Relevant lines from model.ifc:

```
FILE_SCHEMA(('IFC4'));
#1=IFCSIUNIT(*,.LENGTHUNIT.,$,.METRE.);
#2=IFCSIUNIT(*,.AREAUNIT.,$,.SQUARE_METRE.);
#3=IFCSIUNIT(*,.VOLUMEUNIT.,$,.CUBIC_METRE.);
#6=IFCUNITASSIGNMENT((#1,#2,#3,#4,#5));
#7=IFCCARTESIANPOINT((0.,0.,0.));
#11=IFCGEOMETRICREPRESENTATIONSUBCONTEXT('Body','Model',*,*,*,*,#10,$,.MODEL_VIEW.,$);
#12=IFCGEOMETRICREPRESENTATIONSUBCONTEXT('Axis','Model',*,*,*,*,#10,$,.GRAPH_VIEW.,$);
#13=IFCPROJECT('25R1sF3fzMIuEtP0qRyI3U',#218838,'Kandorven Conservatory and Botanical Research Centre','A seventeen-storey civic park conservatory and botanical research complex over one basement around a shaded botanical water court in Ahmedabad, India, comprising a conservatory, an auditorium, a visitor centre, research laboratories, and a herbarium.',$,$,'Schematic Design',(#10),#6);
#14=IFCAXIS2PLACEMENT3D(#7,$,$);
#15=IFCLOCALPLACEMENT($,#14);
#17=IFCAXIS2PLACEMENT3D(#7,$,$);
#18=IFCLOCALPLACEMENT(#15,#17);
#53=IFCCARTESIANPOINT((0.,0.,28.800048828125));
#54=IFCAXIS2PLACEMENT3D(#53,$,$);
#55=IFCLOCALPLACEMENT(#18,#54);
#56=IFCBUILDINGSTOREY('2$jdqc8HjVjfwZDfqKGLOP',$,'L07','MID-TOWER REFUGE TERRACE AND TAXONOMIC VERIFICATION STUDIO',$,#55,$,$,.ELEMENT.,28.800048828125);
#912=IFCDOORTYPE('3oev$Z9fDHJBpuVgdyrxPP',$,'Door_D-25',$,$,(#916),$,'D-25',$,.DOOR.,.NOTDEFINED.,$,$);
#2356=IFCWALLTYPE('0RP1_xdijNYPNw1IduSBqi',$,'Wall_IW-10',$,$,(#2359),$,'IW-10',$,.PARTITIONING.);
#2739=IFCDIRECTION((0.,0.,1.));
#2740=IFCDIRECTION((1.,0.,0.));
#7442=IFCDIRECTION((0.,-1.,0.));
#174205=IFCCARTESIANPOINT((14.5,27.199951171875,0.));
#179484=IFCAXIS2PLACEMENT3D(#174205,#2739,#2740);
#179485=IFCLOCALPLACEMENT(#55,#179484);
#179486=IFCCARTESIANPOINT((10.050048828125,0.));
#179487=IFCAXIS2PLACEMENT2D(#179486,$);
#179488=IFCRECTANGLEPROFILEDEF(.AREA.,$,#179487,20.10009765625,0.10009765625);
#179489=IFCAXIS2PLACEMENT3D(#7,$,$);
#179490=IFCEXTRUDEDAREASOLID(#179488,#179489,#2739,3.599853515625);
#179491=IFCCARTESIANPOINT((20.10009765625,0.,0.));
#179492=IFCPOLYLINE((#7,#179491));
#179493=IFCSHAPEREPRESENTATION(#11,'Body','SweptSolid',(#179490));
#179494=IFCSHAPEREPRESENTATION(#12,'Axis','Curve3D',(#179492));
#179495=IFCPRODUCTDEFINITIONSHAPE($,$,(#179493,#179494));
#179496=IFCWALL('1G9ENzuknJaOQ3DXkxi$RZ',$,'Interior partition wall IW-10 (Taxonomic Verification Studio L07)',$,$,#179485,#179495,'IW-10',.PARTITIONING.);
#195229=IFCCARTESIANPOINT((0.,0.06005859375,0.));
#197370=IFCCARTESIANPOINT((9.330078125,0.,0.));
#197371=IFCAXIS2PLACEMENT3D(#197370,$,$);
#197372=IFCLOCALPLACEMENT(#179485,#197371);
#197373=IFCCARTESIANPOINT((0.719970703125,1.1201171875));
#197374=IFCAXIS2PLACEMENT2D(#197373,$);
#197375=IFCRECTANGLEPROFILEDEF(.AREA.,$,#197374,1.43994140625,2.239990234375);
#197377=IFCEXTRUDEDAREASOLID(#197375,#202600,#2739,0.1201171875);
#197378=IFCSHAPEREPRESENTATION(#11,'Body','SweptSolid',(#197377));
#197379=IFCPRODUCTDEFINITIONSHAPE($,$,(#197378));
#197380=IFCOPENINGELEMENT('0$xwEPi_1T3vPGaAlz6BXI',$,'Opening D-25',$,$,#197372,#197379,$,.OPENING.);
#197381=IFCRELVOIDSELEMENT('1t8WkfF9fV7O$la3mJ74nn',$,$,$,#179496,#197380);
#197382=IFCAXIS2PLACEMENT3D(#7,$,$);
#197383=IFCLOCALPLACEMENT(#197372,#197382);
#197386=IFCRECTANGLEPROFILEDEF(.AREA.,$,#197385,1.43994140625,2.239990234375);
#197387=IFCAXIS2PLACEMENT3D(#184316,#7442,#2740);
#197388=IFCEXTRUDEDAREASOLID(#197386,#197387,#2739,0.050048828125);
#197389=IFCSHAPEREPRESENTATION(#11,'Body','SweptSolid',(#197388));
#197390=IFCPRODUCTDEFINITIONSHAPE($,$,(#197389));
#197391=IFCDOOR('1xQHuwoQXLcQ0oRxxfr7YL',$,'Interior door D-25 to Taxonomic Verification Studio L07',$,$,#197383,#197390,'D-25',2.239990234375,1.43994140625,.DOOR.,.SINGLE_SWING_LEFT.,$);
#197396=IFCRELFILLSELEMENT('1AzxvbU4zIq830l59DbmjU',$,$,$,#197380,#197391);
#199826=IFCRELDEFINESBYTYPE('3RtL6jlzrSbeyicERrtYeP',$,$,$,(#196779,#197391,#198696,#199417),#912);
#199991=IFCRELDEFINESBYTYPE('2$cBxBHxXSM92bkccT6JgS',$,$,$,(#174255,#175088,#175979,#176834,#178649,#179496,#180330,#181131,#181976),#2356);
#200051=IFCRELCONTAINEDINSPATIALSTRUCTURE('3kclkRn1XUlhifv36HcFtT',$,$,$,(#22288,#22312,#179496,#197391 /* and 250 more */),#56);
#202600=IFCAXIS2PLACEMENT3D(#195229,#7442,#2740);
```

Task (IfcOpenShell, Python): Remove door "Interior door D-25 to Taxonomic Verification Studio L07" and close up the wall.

```python
import ifcopenshell
import ifcopenshell.api.feature
import ifcopenshell.api.root
import ifcopenshell.geom
import ifcopenshell.util.shape

model = ifcopenshell.open("model.ifc")
settings = ifcopenshell.geom.settings()


def volume(element):
    """Net volume in cubic metres, openings subtracted."""
    shape = ifcopenshell.geom.create_shape(settings, element)
    return ifcopenshell.util.shape.get_volume(shape.geometry)


door = model.by_guid("1xQHuwoQXLcQ0oRxxfr7YL")
opening = door.FillsVoids[0].RelatingOpeningElement
wall = opening.VoidsElements[0].RelatingBuildingElement
before = volume(wall)

ifcopenshell.api.root.remove_product(model, product=door)
ifcopenshell.api.feature.remove_feature(model, feature=opening)

after = volume(wall)

print(f"wall volume {before:.3f} -> {after:.3f} m3")

model.write("model_rev.ifc")
```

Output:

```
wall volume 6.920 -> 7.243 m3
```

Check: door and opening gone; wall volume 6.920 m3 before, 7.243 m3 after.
